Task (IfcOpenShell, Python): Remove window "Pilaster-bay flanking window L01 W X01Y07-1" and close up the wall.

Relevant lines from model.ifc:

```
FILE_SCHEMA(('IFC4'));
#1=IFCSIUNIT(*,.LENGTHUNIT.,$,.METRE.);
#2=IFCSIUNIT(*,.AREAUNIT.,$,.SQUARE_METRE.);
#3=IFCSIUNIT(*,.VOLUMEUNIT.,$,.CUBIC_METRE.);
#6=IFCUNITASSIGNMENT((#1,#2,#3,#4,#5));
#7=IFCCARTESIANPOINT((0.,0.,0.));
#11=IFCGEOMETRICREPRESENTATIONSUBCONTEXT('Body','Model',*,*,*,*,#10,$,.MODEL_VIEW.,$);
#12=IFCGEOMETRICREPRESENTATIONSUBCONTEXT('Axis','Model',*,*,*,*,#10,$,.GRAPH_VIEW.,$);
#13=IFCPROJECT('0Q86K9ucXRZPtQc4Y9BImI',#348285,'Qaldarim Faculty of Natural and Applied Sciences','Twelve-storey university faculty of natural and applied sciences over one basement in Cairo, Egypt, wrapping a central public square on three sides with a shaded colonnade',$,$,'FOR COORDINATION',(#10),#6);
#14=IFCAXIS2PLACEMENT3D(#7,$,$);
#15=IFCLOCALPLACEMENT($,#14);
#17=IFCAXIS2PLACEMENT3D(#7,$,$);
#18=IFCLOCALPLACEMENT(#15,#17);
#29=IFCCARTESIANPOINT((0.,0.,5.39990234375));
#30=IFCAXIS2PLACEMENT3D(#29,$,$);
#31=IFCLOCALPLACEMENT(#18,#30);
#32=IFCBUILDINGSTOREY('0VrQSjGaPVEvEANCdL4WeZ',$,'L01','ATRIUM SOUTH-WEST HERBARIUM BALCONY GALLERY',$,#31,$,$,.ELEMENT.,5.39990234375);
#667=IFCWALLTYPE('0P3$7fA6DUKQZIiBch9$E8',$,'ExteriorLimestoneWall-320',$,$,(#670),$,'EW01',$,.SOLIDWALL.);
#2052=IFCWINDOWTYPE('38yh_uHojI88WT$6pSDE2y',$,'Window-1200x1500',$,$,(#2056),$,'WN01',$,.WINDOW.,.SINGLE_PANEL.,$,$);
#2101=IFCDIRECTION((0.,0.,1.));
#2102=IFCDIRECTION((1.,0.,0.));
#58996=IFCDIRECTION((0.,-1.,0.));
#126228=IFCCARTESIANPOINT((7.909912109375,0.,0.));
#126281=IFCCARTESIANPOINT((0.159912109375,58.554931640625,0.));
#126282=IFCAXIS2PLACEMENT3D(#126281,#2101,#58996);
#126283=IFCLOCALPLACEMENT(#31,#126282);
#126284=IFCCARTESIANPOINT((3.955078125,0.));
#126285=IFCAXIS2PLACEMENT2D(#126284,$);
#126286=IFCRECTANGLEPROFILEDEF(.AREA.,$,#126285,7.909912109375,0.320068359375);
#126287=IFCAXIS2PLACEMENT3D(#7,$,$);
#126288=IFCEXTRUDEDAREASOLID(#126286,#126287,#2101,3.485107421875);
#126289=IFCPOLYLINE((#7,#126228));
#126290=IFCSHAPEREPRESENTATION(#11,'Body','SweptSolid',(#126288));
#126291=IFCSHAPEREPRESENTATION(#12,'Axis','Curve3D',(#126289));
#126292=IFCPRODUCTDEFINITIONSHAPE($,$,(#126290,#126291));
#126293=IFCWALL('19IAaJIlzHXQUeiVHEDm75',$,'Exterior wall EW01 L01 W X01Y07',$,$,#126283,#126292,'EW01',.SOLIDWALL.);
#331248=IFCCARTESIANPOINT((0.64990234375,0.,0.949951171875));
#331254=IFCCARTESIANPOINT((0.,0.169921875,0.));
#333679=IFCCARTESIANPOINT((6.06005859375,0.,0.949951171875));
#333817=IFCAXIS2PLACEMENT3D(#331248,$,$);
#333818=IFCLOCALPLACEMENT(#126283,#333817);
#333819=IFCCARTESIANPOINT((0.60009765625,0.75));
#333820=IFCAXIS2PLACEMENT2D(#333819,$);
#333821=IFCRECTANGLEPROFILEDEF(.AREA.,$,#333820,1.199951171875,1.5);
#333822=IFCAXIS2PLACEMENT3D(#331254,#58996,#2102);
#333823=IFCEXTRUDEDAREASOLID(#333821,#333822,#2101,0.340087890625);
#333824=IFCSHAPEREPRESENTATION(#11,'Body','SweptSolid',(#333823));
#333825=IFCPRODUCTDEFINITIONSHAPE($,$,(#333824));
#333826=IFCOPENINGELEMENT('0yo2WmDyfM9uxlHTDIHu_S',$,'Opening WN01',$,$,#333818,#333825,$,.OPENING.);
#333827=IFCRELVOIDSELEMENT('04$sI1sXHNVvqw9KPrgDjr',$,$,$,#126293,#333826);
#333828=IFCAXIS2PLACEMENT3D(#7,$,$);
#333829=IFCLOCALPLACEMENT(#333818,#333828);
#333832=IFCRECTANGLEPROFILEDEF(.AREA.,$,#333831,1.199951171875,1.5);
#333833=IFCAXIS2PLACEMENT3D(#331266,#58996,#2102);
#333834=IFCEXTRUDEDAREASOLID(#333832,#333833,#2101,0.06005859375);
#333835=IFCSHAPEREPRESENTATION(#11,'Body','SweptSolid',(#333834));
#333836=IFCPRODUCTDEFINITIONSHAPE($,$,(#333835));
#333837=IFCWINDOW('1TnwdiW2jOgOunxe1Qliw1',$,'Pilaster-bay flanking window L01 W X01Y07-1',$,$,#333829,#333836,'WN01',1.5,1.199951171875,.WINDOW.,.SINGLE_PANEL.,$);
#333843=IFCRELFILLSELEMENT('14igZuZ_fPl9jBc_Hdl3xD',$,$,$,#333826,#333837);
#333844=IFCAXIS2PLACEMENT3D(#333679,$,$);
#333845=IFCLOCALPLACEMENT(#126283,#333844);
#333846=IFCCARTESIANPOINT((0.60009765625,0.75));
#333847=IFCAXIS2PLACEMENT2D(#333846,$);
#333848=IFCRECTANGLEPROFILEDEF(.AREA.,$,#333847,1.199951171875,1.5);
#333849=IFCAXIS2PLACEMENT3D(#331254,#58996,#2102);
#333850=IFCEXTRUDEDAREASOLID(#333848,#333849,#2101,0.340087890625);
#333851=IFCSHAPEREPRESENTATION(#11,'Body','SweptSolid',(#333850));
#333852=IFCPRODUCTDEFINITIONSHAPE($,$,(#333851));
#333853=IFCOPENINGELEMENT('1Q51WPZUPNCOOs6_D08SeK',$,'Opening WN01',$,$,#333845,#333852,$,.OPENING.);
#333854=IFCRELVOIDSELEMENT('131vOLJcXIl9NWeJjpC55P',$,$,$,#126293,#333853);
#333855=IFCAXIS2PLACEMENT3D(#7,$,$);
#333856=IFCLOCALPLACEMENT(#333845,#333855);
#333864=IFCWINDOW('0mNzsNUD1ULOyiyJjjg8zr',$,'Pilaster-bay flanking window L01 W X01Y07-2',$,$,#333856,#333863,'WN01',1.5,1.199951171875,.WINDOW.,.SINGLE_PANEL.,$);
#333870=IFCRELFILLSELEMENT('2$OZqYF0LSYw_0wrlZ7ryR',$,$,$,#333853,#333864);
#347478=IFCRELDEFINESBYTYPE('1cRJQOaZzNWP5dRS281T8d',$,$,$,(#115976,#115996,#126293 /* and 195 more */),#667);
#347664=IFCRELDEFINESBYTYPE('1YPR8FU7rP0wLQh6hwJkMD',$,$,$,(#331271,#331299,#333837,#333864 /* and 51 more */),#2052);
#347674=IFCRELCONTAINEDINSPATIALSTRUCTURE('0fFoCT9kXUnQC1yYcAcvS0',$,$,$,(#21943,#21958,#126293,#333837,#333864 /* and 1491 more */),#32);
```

```python
import ifcopenshell
import ifcopenshell.api.feature
import ifcopenshell.api.root
import ifcopenshell.geom
import ifcopenshell.util.shape

model = ifcopenshell.open("model.ifc")
settings = ifcopenshell.geom.settings()


def volume(element):
    """Net volume in cubic metres, openings subtracted."""
    shape = ifcopenshell.geom.create_shape(settings, element)
    return ifcopenshell.util.shape.get_volume(shape.geometry)


window = model.by_guid("1TnwdiW2jOgOunxe1Qliw1")
opening = window.FillsVoids[0].RelatingOpeningElement
wall = opening.VoidsElements[0].RelatingBuildingElement
before = volume(wall)

ifcopenshell.api.root.remove_product(model, product=window)
ifcopenshell.api.feature.remove_feature(model, feature=opening)

after = volume(wall)

print(f"wall volume {before:.3f} -> {after:.3f} m3")

model.write("model_updated.ifc")
```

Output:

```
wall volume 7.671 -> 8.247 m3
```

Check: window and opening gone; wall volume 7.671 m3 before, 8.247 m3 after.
